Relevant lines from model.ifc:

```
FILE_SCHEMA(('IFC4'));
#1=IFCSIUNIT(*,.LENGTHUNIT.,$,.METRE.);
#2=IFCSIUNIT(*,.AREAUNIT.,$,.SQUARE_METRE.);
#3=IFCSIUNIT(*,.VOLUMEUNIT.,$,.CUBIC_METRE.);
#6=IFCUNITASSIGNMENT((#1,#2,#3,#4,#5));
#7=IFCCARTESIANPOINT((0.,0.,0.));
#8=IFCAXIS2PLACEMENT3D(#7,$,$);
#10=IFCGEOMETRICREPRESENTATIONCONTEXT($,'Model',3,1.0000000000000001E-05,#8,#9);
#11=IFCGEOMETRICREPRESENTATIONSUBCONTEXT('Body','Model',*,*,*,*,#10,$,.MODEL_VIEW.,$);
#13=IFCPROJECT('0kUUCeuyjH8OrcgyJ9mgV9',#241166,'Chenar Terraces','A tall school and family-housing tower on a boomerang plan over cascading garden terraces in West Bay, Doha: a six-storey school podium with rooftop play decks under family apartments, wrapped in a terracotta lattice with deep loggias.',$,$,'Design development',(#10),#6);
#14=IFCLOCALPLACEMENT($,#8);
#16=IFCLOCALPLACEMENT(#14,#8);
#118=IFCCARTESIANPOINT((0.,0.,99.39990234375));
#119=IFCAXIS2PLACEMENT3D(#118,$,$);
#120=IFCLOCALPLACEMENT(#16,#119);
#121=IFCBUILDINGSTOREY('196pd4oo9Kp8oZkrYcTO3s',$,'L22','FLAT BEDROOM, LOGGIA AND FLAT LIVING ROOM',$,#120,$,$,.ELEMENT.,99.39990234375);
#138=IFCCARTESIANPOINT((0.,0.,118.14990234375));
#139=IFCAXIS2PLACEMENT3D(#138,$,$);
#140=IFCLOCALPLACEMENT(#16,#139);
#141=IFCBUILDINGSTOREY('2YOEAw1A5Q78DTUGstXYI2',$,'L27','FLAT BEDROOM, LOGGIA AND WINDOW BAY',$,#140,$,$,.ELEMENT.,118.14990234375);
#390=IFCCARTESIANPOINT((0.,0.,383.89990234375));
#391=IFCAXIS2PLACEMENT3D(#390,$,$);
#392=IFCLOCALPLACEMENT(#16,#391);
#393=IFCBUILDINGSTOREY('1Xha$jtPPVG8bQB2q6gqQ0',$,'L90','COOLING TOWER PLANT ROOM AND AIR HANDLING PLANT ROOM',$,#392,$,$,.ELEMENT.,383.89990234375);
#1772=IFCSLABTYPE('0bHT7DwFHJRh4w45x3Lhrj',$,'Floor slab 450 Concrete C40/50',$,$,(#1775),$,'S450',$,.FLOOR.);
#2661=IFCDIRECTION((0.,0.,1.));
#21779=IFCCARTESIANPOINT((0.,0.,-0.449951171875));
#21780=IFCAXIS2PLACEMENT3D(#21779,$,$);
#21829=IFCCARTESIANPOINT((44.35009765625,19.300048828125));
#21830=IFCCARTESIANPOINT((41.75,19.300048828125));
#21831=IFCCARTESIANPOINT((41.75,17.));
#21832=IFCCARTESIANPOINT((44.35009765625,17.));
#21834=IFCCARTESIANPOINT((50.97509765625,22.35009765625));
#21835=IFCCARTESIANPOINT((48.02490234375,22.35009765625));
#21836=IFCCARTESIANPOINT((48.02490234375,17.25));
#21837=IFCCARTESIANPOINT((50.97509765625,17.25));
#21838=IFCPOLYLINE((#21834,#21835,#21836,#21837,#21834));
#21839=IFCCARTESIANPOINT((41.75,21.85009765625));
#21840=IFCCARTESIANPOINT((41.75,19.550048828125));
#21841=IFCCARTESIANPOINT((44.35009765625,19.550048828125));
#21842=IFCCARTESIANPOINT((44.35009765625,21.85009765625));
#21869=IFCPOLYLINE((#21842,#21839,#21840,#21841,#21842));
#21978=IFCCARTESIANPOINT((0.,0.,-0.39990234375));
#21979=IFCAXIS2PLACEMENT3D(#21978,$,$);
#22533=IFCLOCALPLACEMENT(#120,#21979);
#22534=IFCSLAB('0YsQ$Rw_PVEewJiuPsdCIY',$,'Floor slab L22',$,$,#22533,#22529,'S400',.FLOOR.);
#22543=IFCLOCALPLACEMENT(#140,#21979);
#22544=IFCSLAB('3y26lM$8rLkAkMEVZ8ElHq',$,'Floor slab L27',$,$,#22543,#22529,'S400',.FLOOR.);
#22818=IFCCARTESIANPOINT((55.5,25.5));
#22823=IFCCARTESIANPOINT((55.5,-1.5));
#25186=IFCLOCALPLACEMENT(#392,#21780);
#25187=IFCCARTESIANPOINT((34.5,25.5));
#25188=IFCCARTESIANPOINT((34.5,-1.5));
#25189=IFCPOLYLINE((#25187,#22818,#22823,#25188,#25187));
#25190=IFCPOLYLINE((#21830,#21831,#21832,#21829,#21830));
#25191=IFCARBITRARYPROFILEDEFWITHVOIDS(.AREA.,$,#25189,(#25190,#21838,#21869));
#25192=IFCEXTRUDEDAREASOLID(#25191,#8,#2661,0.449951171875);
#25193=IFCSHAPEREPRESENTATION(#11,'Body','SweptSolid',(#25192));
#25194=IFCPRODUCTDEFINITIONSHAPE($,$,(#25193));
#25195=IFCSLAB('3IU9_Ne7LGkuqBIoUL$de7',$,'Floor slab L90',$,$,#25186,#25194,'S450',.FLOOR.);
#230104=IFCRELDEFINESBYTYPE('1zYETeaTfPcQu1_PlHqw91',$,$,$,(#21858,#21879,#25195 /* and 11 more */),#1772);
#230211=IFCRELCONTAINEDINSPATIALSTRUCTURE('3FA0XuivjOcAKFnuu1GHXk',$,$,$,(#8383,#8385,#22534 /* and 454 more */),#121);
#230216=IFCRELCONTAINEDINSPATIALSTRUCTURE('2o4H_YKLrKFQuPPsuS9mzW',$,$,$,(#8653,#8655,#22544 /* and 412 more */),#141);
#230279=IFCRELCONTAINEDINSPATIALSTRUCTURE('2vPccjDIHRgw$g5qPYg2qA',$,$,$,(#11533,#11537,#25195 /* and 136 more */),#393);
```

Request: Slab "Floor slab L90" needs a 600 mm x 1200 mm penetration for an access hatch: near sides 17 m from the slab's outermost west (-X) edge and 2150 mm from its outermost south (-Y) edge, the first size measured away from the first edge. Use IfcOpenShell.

```python
import numpy as np
import ifcopenshell
import ifcopenshell.api.feature
import ifcopenshell.api.geometry
import ifcopenshell.api.root
import ifcopenshell.geom
import ifcopenshell.util.placement
import ifcopenshell.util.representation
import ifcopenshell.util.shape
import ifcopenshell.util.unit

model = ifcopenshell.open("model.ifc")
unit_scale = ifcopenshell.util.unit.calculate_unit_scale(model)
settings = ifcopenshell.geom.settings()


def volume(element):
    """Net volume in cubic metres, openings subtracted."""
    shape = ifcopenshell.geom.create_shape(settings, element)
    return ifcopenshell.util.shape.get_volume(shape.geometry)


slab = model.by_guid("3IU9_Ne7LGkuqBIoUL$de7")
before = volume(slab)

# Extent in the slab's own axes, in metres. The edges named are its -X and -Y sides.
slab_shape = ifcopenshell.geom.create_shape(settings, slab)
vertices = ifcopenshell.util.shape.get_vertices(slab_shape.geometry)
x_min, y_min, bottom = vertices.min(axis=0)
top = vertices[:, 2].max()

opening = ifcopenshell.api.root.create_entity(model, ifc_class="IfcOpeningElement", name="Access hatch opening", predefined_type="OPENING")
context = ifcopenshell.util.representation.get_context(model, "Model", "Body", "MODEL_VIEW")
width, depth = 0.6, 1.2
outline = [(0.0, 0.0), (width, 0.0), (width, depth), (0.0, depth), (0.0, 0.0)]
# Overshoot both faces by 50 mm so the cut is clean.
shape = ifcopenshell.api.geometry.add_slab_representation(
    model, context=context, depth=top - bottom + 0.1, polyline=outline
)
ifcopenshell.api.geometry.assign_representation(model, product=opening, representation=shape)

matrix = ifcopenshell.util.placement.get_local_placement(slab.ObjectPlacement)
matrix[:, 3] = matrix @ np.append(np.array([x_min + 17, y_min + 2.15, bottom - 0.05]) / unit_scale, 1.0)
ifcopenshell.api.geometry.edit_object_placement(model, product=opening, matrix=matrix, is_si=False)
ifcopenshell.api.feature.add_feature(model, feature=opening, element=slab)

after = volume(slab)

print(f"slab volume {before:.3f} -> {after:.3f} m3")

model.write("model_rev.ifc")
```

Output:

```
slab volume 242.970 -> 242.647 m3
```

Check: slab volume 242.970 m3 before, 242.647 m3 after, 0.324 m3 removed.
